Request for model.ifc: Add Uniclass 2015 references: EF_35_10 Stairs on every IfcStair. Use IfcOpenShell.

First a look at what the model holds.

```python
import ifcopenshell

model = ifcopenshell.open("model.ifc")
print(model.schema)
print("classifications:", [c.Name for c in model.by_type("IfcClassification")])
for ifc_class in ("IfcDoor", "IfcRoof", "IfcStair", "IfcWall", "IfcWindow"):
    print(ifc_class, len(model.by_type(ifc_class)))
```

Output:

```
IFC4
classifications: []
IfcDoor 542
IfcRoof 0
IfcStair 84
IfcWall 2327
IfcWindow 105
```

```python
import ifcopenshell
import ifcopenshell.api.classification

model = ifcopenshell.open("model.ifc")

system = ifcopenshell.api.classification.add_classification(model, classification="Uniclass 2015")

codes = {
    "IfcStair": ("EF_35_10", "Stairs"),
}
for ifc_class, (code, name) in codes.items():
    products = model.by_type(ifc_class)
    ifcopenshell.api.classification.add_reference(
        model, products=products, classification=system, identification=code, name=name
    )
    print(code, len(products))

model.write("model-out.ifc")
```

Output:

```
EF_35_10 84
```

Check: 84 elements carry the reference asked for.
